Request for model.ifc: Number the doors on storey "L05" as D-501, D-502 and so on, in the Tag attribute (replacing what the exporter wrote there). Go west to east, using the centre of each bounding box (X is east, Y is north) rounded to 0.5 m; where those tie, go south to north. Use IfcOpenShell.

First a look at what the model holds.

```python
import ifcopenshell
import ifcopenshell.util.element
import ifcopenshell.util.placement

model = ifcopenshell.open("model.ifc")
print(model.schema)
storey = next(s for s in model.by_type("IfcBuildingStorey") if s.Name == "L05")
doors = [e for e in ifcopenshell.util.element.get_decomposition(storey) if e.is_a("IfcDoor")]
for e in sorted(doors, key=lambda e: e.id()):
    origin = ifcopenshell.util.placement.get_local_placement(e.ObjectPlacement)[:3, 3]
    print(e.id(), e.Tag, e.Name, origin.round(2) + 0.0, sep=" | ")
```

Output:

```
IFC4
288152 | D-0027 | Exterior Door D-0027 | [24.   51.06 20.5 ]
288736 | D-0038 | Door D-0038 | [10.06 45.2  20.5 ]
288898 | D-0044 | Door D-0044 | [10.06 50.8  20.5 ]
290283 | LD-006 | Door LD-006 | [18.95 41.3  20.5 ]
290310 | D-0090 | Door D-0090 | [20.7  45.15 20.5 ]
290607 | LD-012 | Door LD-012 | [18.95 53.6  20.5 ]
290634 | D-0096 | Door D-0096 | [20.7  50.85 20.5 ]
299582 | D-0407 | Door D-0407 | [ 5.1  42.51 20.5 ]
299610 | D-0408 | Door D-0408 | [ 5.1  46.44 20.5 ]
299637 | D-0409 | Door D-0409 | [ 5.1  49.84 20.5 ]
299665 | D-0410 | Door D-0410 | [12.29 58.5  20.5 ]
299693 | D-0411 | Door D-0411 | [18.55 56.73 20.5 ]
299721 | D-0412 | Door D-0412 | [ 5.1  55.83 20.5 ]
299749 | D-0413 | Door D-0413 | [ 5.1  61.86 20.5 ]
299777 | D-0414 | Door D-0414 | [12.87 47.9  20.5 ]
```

```python
import ifcopenshell
import ifcopenshell.geom
import ifcopenshell.util.element
import ifcopenshell.util.shape

model = ifcopenshell.open("model.ifc")
settings = ifcopenshell.geom.settings()
settings.set("use-world-coords", True)


def centre(element):
    shape = ifcopenshell.geom.create_shape(settings, element)
    return ifcopenshell.util.shape.get_bbox_centroid(shape.geometry)


storey = next(s for s in model.by_type("IfcBuildingStorey") if s.Name == "L05")
doors = [e for e in ifcopenshell.util.element.get_decomposition(storey) if e.is_a("IfcDoor")]

# Insertion points can sit at a corner or the storey origin, so sort by the geometry (in metres).
centres = {e: centre(e) for e in doors}
doors.sort(key=lambda e: (round(centres[e][0] / 0.5), centres[e][1]))

for i, e in enumerate(doors, start=1):
    number = f"D-5{i:02d}"
    e.Tag = number
    print(e.id(), number)

model.write("model_rev.ifc")
```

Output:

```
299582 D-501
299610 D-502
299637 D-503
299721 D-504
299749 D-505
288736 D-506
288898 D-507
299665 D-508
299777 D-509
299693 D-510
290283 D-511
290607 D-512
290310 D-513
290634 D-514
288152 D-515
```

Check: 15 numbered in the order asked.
